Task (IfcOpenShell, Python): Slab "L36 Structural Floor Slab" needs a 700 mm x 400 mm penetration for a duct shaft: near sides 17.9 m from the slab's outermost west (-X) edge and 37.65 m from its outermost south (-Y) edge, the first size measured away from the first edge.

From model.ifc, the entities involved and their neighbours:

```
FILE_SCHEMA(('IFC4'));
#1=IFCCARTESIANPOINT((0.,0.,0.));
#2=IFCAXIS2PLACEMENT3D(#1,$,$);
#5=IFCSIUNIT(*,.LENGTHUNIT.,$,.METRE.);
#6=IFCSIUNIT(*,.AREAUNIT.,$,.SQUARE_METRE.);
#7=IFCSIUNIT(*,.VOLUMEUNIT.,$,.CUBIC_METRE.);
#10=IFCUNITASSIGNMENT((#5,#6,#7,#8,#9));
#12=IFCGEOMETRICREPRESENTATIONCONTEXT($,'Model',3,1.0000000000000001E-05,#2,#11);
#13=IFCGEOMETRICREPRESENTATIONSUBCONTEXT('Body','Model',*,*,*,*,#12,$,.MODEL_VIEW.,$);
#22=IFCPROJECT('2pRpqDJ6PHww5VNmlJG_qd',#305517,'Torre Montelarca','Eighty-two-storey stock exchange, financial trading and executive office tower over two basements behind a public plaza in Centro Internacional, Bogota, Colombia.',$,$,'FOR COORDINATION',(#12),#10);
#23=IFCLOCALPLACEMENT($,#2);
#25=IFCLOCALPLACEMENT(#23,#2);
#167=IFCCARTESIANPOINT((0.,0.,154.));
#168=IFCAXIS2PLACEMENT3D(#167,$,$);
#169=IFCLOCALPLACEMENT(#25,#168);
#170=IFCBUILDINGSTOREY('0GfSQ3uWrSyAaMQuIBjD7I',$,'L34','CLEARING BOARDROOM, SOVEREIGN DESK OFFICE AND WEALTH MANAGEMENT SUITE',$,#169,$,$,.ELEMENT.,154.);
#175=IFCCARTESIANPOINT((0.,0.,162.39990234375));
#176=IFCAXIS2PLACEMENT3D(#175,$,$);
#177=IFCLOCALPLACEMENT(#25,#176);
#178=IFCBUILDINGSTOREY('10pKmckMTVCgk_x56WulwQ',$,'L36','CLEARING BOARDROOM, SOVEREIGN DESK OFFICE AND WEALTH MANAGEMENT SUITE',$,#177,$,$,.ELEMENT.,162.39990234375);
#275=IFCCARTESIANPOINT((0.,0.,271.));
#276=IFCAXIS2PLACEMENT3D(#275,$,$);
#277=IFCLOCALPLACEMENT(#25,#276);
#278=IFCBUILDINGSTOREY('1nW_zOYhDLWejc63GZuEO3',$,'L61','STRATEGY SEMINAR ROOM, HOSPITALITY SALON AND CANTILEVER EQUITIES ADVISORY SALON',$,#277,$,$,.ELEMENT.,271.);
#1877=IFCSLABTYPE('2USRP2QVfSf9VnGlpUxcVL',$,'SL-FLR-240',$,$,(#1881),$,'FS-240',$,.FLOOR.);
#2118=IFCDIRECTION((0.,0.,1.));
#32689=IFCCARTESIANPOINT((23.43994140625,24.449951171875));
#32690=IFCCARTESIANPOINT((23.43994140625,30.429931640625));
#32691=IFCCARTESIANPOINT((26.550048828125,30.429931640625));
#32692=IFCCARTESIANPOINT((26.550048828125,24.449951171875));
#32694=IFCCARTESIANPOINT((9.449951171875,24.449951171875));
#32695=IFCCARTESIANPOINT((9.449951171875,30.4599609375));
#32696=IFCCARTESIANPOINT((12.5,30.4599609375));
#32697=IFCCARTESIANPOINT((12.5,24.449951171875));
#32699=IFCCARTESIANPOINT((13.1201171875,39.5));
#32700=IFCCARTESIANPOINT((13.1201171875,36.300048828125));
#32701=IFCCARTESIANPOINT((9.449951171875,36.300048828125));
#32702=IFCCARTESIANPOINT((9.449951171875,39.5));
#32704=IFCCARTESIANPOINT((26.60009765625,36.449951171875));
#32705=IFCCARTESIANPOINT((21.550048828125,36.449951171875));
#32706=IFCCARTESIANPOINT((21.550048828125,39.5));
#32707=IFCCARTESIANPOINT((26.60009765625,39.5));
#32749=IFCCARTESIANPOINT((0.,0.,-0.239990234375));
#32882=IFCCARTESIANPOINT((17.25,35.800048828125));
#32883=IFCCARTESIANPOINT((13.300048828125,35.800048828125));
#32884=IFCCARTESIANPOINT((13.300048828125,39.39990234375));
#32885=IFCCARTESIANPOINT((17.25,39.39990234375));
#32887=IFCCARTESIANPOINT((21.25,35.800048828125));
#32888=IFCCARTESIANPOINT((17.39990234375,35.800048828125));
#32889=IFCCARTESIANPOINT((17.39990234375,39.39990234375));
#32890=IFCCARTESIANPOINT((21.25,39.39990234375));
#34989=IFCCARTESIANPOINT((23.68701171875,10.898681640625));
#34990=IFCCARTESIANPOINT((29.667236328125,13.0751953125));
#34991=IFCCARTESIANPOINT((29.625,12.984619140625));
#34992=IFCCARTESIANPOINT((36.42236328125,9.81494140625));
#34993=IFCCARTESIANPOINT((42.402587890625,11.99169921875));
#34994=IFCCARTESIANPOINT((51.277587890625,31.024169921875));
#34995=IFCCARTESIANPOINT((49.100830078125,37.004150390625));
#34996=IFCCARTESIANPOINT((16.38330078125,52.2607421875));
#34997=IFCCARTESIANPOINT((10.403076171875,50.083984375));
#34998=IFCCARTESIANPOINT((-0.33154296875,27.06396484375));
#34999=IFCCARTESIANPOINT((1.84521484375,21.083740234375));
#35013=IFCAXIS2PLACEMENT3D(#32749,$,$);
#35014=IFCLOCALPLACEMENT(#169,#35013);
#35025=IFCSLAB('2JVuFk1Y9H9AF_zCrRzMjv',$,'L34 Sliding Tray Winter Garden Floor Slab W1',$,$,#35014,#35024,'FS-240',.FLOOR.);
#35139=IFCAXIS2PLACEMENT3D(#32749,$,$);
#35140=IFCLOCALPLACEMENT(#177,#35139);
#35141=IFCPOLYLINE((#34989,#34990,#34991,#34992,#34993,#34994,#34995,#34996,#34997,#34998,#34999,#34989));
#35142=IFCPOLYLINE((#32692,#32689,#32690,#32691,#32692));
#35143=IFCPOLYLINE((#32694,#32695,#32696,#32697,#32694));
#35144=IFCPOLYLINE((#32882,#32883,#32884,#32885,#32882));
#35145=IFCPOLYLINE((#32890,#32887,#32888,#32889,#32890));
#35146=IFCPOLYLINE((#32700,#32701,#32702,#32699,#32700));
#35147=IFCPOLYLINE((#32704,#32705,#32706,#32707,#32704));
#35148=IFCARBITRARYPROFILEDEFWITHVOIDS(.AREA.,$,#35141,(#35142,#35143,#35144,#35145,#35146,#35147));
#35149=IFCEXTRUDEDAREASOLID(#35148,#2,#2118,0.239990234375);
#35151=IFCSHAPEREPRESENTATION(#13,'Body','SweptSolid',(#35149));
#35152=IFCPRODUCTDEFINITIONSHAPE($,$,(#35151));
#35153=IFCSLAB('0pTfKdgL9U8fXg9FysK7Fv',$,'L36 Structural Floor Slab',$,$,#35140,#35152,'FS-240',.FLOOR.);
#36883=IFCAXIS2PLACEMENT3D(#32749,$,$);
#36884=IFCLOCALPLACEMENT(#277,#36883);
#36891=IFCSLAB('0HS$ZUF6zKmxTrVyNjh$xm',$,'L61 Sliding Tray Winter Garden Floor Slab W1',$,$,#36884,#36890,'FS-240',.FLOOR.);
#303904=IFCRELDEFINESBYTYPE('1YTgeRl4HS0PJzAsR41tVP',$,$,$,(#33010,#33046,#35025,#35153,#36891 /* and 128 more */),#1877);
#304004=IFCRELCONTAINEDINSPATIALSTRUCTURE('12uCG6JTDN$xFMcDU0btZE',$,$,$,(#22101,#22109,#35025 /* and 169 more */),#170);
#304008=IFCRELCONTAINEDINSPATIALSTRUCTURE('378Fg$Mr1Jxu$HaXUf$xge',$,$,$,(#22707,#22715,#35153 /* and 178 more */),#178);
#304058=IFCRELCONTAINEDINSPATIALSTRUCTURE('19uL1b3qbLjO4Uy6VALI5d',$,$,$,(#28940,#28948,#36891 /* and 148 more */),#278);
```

```python
import numpy as np
import ifcopenshell
import ifcopenshell.api.feature
import ifcopenshell.api.geometry
import ifcopenshell.api.root
import ifcopenshell.geom
import ifcopenshell.util.placement
import ifcopenshell.util.representation
import ifcopenshell.util.shape
import ifcopenshell.util.unit

model = ifcopenshell.open("model.ifc")
unit_scale = ifcopenshell.util.unit.calculate_unit_scale(model)
settings = ifcopenshell.geom.settings()


def volume(element):
    """Net volume in cubic metres, openings subtracted."""
    shape = ifcopenshell.geom.create_shape(settings, element)
    return ifcopenshell.util.shape.get_volume(shape.geometry)


slab = model.by_guid("0pTfKdgL9U8fXg9FysK7Fv")
before = volume(slab)

# Extent in the slab's own axes, in metres. The edges named are its -X and -Y sides.
slab_shape = ifcopenshell.geom.create_shape(settings, slab)
vertices = ifcopenshell.util.shape.get_vertices(slab_shape.geometry)
x_min, y_min, bottom = vertices.min(axis=0)
top = vertices[:, 2].max()

opening = ifcopenshell.api.root.create_entity(model, ifc_class="IfcOpeningElement", name="Duct shaft opening", predefined_type="OPENING")
context = ifcopenshell.util.representation.get_context(model, "Model", "Body", "MODEL_VIEW")
width, depth = 0.7, 0.4
outline = [(0.0, 0.0), (width, 0.0), (width, depth), (0.0, depth), (0.0, 0.0)]
# Overshoot both faces by 50 mm so the cut is clean.
shape = ifcopenshell.api.geometry.add_slab_representation(
    model, context=context, depth=top - bottom + 0.1, polyline=outline
)
ifcopenshell.api.geometry.assign_representation(model, product=opening, representation=shape)

matrix = ifcopenshell.util.placement.get_local_placement(slab.ObjectPlacement)
matrix[:, 3] = matrix @ np.append(np.array([x_min + 17.9, y_min + 37.65, bottom - 0.05]) / unit_scale, 1.0)
ifcopenshell.api.geometry.edit_object_placement(model, product=opening, matrix=matrix, is_si=False)
ifcopenshell.api.feature.add_feature(model, feature=opening, element=slab)

after = volume(slab)

print(f"slab volume {before:.3f} -> {after:.3f} m3")

model.write("model_updated.ifc")
```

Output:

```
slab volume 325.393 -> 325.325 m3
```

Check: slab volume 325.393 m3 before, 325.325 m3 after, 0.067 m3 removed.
